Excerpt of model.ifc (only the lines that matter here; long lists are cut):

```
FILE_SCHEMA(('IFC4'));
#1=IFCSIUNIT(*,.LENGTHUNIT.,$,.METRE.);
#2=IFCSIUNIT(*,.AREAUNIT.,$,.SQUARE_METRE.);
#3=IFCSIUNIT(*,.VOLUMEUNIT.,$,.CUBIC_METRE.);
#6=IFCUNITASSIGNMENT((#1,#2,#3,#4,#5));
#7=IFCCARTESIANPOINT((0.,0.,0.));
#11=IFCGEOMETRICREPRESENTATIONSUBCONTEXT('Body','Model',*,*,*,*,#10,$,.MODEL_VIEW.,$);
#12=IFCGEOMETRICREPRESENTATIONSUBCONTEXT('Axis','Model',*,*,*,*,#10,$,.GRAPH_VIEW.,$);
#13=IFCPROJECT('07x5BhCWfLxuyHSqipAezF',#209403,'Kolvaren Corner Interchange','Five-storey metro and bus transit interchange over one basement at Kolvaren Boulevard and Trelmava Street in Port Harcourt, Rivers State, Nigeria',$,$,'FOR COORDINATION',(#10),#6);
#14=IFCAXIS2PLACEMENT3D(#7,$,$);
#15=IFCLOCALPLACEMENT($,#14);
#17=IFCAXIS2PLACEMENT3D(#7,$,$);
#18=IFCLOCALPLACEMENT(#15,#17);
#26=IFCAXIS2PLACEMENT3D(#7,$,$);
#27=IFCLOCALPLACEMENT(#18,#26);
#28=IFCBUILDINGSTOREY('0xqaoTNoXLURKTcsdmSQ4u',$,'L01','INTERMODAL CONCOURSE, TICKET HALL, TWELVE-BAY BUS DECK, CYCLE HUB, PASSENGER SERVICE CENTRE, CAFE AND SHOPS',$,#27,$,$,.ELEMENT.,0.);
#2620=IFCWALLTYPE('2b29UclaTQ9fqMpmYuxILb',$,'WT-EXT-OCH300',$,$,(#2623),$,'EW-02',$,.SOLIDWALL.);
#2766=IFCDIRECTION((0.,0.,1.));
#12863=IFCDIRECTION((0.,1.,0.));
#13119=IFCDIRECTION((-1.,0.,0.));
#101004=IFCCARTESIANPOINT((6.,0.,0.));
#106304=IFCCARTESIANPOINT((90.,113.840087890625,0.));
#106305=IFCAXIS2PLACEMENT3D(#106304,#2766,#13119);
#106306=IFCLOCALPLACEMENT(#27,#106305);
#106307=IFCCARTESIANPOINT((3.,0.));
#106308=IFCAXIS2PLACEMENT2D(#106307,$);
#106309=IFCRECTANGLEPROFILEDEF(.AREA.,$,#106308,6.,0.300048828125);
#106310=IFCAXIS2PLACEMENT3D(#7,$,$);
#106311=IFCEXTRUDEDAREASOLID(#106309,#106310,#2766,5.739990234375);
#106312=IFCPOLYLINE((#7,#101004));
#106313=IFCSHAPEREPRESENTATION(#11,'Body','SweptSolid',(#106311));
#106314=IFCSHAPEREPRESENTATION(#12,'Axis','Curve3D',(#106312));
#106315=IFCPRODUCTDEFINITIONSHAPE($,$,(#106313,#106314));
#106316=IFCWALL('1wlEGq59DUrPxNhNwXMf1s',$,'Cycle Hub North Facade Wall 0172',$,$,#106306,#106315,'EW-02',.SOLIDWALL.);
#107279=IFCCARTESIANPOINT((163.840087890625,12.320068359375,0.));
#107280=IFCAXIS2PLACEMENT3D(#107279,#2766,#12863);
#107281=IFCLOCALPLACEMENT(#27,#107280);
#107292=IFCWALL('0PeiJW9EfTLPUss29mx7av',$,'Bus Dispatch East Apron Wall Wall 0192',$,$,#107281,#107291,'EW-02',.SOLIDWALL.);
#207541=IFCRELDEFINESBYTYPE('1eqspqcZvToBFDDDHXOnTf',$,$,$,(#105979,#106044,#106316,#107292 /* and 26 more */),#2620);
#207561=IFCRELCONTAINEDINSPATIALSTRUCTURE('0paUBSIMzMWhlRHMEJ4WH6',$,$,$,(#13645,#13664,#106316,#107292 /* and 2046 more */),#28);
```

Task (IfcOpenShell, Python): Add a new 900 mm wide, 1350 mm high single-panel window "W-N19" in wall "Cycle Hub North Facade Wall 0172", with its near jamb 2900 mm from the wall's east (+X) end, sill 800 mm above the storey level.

```python
import numpy as np
import ifcopenshell
import ifcopenshell.api.feature
import ifcopenshell.api.geometry
import ifcopenshell.api.root
import ifcopenshell.api.spatial
import ifcopenshell.geom
import ifcopenshell.util.element
import ifcopenshell.util.placement
import ifcopenshell.util.representation
import ifcopenshell.util.shape
import ifcopenshell.util.unit

model = ifcopenshell.open("model.ifc")
unit_scale = ifcopenshell.util.unit.calculate_unit_scale(model)
settings = ifcopenshell.geom.settings()


def volume(element):
    """Net volume in cubic metres, openings subtracted."""
    shape = ifcopenshell.geom.create_shape(settings, element)
    return ifcopenshell.util.shape.get_volume(shape.geometry)


wall = model.by_guid("1wlEGq59DUrPxNhNwXMf1s")
storey = ifcopenshell.util.element.get_container(wall, ifc_class="IfcBuildingStorey")
context = ifcopenshell.util.representation.get_context(model, "Model", "Body", "MODEL_VIEW")
before = volume(wall)

width, height, from_end, sill = 0.9, 1.35, 2.9, 0.8  # metres

# The wall runs along its own X axis, and the end named is its -X end.
wall_shape = ifcopenshell.geom.create_shape(settings, wall)
x, y, z = ifcopenshell.util.shape.get_vertices(wall_shape.geometry).T
start = x.min() + from_end
face, thickness = float(y.min()), float(y.max() - y.min())
wall_matrix = ifcopenshell.util.placement.get_local_placement(wall.ObjectPlacement)
level = ifcopenshell.util.placement.get_local_placement(storey.ObjectPlacement)[2, 3]


def in_wall(x, y):
    """Placement at x, y metres in the wall's axes, at sill height."""
    matrix = wall_matrix.copy()
    matrix[:, 3] = wall_matrix @ np.array([x / unit_scale, y / unit_scale, 0.0, 1.0])
    matrix[2, 3] = level + sill / unit_scale
    return matrix


# Opening: a box that overshoots both wall faces by 50 mm.
opening = ifcopenshell.api.root.create_entity(model, ifc_class="IfcOpeningElement", predefined_type="OPENING")
box = ifcopenshell.api.geometry.add_wall_representation(
    model, context=context, length=width, height=height, thickness=thickness + 0.1
)
ifcopenshell.api.geometry.assign_representation(model, product=opening, representation=box)
ifcopenshell.api.geometry.edit_object_placement(model, product=opening, matrix=in_wall(start, face - 0.05), is_si=False)
ifcopenshell.api.feature.add_feature(model, feature=opening, element=wall)

window = ifcopenshell.api.root.create_entity(model, ifc_class="IfcWindow", name="W-N19", predefined_type="WINDOW")
window.OverallWidth, window.OverallHeight = width / unit_scale, height / unit_scale
window.PartitioningType = "SINGLE_PANEL"
body = ifcopenshell.api.geometry.add_window_representation(
    model,
    context=context,
    overall_width=window.OverallWidth,
    overall_height=window.OverallHeight,
    partition_type="SINGLE_PANEL",
)
ifcopenshell.api.geometry.assign_representation(model, product=window, representation=body)
ifcopenshell.api.spatial.assign_container(model, products=[window], relating_structure=storey)
ifcopenshell.api.feature.add_filling(model, opening=opening, element=window)

# Centre the window in the wall's thickness.
ifcopenshell.api.geometry.edit_object_placement(model, product=window, matrix=in_wall(start, face), is_si=False)
window_shape = ifcopenshell.geom.create_shape(settings, window)
depth = ifcopenshell.util.shape.get_vertices(window_shape.geometry)[:, 1]
offset = face + thickness / 2 - (depth.min() + depth.max()) / 2
ifcopenshell.api.geometry.edit_object_placement(model, product=window, matrix=in_wall(start, offset), is_si=False)

after = volume(wall)

print(f"wall volume {before:.3f} -> {after:.3f} m3")

model.write("model_updated.ifc")
```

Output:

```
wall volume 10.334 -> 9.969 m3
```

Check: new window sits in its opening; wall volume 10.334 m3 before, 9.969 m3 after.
